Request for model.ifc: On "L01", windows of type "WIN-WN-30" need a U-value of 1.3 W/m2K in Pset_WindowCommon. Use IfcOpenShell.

First a look at what the model holds.

```python
import ifcopenshell
import ifcopenshell.util.element

model = ifcopenshell.open("model.ifc")
print(model.schema)
storey = next(s for s in model.by_type("IfcBuildingStorey") if s.Name == "L01")
windows = [e for e in ifcopenshell.util.element.get_decomposition(storey) if e.is_a("IfcWindow")]
seen = {}
for e in windows:
    element_type = ifcopenshell.util.element.get_type(e)
    key = (element_type.Name if element_type != e and element_type else None, ifcopenshell.util.element.get_pset(e, "Pset_WindowCommon", "ThermalTransmittance"))
    seen[key] = seen.get(key, 0) + 1
for (name, value), count in sorted(seen.items(), key=str):
    print(count, "x", name, "|", value)
```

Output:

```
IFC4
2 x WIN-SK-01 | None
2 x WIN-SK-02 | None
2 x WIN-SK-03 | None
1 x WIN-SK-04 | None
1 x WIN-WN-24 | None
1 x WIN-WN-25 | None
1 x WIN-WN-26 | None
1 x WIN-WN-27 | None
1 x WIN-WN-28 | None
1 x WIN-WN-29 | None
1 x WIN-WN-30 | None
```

```python
import ifcopenshell
import ifcopenshell.api.pset
import ifcopenshell.util.element

model = ifcopenshell.open("model.ifc")

storey = next(s for s in model.by_type("IfcBuildingStorey") if s.Name == "L01")
windows = [e for e in ifcopenshell.util.element.get_decomposition(storey) if e.is_a("IfcWindow")]

count = 0
for e in windows:
    element_type = ifcopenshell.util.element.get_type(e)
    if element_type in (None, e) or element_type.Name != "WIN-WN-30":
        continue
    # add_pset returns the element's existing set when there is one.
    pset = ifcopenshell.api.pset.add_pset(model, product=e, name="Pset_WindowCommon")
    ifcopenshell.api.pset.edit_pset(model, pset=pset, properties={"ThermalTransmittance": 1.3})
    count += 1

print(count, "windows updated")

model.write("model_v2.ifc")
```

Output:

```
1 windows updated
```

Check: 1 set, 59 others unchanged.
